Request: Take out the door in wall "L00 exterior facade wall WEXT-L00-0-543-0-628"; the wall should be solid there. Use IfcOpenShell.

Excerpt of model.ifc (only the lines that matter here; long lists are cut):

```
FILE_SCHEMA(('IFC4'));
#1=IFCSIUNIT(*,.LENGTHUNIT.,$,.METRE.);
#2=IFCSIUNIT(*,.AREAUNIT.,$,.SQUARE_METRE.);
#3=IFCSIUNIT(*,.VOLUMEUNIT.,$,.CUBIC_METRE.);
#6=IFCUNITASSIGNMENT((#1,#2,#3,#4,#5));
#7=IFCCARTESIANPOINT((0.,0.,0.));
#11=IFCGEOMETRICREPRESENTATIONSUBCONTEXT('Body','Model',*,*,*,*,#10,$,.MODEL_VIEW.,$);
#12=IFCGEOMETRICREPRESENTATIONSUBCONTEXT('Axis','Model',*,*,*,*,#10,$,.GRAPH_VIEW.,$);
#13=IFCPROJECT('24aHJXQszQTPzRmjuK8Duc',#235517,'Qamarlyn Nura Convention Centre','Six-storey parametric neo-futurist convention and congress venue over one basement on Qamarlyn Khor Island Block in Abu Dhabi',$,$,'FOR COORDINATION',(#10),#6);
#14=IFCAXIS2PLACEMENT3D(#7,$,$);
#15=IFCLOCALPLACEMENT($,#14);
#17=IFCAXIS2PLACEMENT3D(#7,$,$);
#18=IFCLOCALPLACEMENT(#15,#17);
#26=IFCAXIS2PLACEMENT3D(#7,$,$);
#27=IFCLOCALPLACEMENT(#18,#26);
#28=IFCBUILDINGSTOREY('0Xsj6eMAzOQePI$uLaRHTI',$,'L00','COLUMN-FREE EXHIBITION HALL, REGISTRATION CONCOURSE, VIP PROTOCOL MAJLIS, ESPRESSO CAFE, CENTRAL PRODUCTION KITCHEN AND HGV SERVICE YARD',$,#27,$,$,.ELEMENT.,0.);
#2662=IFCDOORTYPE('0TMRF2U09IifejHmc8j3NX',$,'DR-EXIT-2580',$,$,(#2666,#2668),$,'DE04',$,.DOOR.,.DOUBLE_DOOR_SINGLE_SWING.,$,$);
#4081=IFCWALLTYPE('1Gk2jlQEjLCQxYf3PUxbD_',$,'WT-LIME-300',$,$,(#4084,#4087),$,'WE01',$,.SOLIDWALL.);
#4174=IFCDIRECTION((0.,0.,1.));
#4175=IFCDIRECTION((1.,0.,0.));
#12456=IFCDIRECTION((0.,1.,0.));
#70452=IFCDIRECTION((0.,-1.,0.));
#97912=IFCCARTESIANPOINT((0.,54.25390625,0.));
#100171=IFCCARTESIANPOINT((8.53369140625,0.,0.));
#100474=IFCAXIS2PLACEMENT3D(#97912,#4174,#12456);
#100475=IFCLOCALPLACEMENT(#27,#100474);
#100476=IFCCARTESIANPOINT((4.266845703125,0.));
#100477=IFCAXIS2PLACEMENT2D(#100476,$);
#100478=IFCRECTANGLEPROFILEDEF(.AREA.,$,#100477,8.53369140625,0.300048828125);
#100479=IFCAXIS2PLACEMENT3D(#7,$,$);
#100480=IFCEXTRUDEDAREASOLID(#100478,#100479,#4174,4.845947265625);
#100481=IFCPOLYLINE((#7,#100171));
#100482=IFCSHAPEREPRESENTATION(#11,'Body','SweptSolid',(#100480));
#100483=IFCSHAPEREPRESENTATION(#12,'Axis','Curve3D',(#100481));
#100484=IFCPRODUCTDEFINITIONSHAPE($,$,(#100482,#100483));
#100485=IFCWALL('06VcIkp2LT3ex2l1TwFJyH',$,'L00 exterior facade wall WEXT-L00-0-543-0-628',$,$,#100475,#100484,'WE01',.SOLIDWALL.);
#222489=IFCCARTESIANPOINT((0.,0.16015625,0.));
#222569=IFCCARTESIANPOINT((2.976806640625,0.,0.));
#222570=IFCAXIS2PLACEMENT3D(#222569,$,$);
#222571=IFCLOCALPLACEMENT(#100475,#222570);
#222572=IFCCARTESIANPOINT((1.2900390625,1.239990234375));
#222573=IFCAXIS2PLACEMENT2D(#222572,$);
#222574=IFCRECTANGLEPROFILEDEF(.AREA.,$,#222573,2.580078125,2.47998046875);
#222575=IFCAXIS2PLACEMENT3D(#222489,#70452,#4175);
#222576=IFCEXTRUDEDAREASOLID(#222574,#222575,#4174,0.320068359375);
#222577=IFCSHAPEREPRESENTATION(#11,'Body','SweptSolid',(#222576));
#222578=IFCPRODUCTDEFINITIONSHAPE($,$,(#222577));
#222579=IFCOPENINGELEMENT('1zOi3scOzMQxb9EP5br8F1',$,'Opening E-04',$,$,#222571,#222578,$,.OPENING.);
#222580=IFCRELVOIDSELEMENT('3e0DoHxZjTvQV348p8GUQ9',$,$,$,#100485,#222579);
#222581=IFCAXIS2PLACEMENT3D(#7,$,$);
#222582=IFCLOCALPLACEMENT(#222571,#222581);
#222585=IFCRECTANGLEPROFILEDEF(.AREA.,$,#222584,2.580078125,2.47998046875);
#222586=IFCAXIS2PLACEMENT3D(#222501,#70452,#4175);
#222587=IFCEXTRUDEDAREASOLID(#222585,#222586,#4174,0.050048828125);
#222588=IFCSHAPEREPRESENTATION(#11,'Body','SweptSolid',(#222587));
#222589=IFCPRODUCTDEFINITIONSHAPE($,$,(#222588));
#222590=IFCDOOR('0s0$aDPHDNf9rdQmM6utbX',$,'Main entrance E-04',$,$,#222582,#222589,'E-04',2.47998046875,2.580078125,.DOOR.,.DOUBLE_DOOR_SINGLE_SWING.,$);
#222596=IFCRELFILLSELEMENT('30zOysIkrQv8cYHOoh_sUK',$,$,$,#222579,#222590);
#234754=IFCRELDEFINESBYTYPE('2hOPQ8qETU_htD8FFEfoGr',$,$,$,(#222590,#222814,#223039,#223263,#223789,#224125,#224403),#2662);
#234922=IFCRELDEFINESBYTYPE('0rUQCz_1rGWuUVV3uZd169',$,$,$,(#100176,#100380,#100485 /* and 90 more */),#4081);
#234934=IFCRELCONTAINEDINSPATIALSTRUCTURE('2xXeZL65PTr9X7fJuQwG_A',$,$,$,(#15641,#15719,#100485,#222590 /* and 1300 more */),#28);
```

```python
import ifcopenshell
import ifcopenshell.api.feature
import ifcopenshell.api.root
import ifcopenshell.geom
import ifcopenshell.util.shape

model = ifcopenshell.open("model.ifc")
settings = ifcopenshell.geom.settings()


def volume(element):
    """Net volume in cubic metres, openings subtracted."""
    shape = ifcopenshell.geom.create_shape(settings, element)
    return ifcopenshell.util.shape.get_volume(shape.geometry)


door = model.by_guid("0s0$aDPHDNf9rdQmM6utbX")
opening = door.FillsVoids[0].RelatingOpeningElement
wall = opening.VoidsElements[0].RelatingBuildingElement
before = volume(wall)

ifcopenshell.api.root.remove_product(model, product=door)
ifcopenshell.api.feature.remove_feature(model, feature=opening)

after = volume(wall)

print(f"wall volume {before:.3f} -> {after:.3f} m3")

model.write("model_v2.ifc")
```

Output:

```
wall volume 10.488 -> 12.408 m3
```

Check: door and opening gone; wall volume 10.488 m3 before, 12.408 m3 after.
